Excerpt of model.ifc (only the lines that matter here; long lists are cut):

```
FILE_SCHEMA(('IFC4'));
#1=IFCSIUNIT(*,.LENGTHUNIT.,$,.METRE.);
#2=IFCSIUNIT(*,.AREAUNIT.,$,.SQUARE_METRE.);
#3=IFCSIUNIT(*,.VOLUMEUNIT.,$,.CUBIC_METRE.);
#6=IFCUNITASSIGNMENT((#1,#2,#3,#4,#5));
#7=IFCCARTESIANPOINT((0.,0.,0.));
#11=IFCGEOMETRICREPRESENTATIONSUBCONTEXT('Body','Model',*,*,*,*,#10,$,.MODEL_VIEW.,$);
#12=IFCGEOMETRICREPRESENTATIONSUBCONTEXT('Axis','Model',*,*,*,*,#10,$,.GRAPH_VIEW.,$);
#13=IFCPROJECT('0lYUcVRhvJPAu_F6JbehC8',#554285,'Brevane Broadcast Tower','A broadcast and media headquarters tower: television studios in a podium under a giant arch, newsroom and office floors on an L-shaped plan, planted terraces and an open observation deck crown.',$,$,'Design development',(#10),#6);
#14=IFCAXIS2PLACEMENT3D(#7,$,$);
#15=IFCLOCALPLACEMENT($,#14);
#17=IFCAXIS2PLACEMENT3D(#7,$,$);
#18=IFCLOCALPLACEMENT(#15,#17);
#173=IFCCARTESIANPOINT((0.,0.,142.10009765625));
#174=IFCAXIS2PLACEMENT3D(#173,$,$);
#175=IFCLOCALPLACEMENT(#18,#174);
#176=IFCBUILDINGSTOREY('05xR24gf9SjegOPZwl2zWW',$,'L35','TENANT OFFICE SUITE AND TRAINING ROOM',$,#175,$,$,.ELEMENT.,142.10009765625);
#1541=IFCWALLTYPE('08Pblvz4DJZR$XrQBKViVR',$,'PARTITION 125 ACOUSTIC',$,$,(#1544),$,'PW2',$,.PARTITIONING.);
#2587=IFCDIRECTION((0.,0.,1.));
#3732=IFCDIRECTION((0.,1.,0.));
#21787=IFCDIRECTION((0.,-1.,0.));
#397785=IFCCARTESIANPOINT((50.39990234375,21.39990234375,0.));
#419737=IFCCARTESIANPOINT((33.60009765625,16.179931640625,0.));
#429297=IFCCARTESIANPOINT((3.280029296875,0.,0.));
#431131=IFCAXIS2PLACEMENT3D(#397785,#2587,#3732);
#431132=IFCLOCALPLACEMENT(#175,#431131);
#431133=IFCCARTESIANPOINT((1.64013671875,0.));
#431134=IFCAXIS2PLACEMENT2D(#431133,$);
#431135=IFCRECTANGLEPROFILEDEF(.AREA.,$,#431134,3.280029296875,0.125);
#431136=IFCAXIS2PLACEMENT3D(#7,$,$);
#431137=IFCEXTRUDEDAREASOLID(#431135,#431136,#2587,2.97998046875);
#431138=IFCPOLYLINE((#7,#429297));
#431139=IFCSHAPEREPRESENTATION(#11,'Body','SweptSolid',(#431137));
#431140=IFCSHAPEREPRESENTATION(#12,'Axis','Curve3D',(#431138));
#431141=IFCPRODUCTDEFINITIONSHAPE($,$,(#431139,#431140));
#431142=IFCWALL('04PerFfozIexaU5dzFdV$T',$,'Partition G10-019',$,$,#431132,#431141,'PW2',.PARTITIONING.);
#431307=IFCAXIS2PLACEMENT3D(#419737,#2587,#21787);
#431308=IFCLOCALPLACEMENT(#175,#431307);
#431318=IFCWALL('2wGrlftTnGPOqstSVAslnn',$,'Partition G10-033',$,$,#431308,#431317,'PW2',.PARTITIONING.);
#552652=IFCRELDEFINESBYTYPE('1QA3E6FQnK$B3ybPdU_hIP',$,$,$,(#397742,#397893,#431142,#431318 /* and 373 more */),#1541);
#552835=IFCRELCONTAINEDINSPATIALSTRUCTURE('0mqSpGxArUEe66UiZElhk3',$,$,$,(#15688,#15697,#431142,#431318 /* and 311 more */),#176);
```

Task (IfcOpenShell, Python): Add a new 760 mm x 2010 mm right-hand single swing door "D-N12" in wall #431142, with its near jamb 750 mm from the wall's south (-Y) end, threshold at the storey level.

```python
import numpy as np
import ifcopenshell
import ifcopenshell.api.feature
import ifcopenshell.api.geometry
import ifcopenshell.api.root
import ifcopenshell.api.spatial
import ifcopenshell.geom
import ifcopenshell.util.element
import ifcopenshell.util.placement
import ifcopenshell.util.representation
import ifcopenshell.util.shape
import ifcopenshell.util.unit

model = ifcopenshell.open("model.ifc")
unit_scale = ifcopenshell.util.unit.calculate_unit_scale(model)
settings = ifcopenshell.geom.settings()


def volume(element):
    """Net volume in cubic metres, openings subtracted."""
    shape = ifcopenshell.geom.create_shape(settings, element)
    return ifcopenshell.util.shape.get_volume(shape.geometry)


wall = model.by_guid("04PerFfozIexaU5dzFdV$T")
storey = ifcopenshell.util.element.get_container(wall, ifc_class="IfcBuildingStorey")
context = ifcopenshell.util.representation.get_context(model, "Model", "Body", "MODEL_VIEW")
before = volume(wall)

width, height, from_end, sill = 0.76, 2.01, 0.75, 0.0  # metres

# The wall runs along its own X axis, and the end named is its -X end.
wall_shape = ifcopenshell.geom.create_shape(settings, wall)
x, y, z = ifcopenshell.util.shape.get_vertices(wall_shape.geometry).T
start = x.min() + from_end
face, thickness = float(y.min()), float(y.max() - y.min())
wall_matrix = ifcopenshell.util.placement.get_local_placement(wall.ObjectPlacement)
level = ifcopenshell.util.placement.get_local_placement(storey.ObjectPlacement)[2, 3]


def in_wall(x, y):
    """Placement at x, y metres in the wall's axes, at sill height."""
    matrix = wall_matrix.copy()
    matrix[:, 3] = wall_matrix @ np.array([x / unit_scale, y / unit_scale, 0.0, 1.0])
    matrix[2, 3] = level + sill / unit_scale
    return matrix


# Opening: a box that overshoots both wall faces by 50 mm.
opening = ifcopenshell.api.root.create_entity(model, ifc_class="IfcOpeningElement", predefined_type="OPENING")
box = ifcopenshell.api.geometry.add_wall_representation(
    model, context=context, length=width, height=height, thickness=thickness + 0.1
)
ifcopenshell.api.geometry.assign_representation(model, product=opening, representation=box)
ifcopenshell.api.geometry.edit_object_placement(model, product=opening, matrix=in_wall(start, face - 0.05), is_si=False)
ifcopenshell.api.feature.add_feature(model, feature=opening, element=wall)

door = ifcopenshell.api.root.create_entity(model, ifc_class="IfcDoor", name="D-N12", predefined_type="DOOR")
door.OverallWidth, door.OverallHeight = width / unit_scale, height / unit_scale
door.OperationType = "SINGLE_SWING_RIGHT"
body = ifcopenshell.api.geometry.add_door_representation(
    model,
    context=context,
    overall_width=door.OverallWidth,
    overall_height=door.OverallHeight,
    operation_type="SINGLE_SWING_RIGHT",
    lining_properties={"LiningDepth": thickness / unit_scale, "ThresholdDepth": thickness / unit_scale},
)
ifcopenshell.api.geometry.assign_representation(model, product=door, representation=body)
ifcopenshell.api.spatial.assign_container(model, products=[door], relating_structure=storey)
ifcopenshell.api.feature.add_filling(model, opening=opening, element=door)

# The lining spans the wall, so the door starts at the wall face.
ifcopenshell.api.geometry.edit_object_placement(model, product=door, matrix=in_wall(start, face), is_si=False)

after = volume(wall)

print(f"wall volume {before:.3f} -> {after:.3f} m3")

model.write("model-out.ifc")
```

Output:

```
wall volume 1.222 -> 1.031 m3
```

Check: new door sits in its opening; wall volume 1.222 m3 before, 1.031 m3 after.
